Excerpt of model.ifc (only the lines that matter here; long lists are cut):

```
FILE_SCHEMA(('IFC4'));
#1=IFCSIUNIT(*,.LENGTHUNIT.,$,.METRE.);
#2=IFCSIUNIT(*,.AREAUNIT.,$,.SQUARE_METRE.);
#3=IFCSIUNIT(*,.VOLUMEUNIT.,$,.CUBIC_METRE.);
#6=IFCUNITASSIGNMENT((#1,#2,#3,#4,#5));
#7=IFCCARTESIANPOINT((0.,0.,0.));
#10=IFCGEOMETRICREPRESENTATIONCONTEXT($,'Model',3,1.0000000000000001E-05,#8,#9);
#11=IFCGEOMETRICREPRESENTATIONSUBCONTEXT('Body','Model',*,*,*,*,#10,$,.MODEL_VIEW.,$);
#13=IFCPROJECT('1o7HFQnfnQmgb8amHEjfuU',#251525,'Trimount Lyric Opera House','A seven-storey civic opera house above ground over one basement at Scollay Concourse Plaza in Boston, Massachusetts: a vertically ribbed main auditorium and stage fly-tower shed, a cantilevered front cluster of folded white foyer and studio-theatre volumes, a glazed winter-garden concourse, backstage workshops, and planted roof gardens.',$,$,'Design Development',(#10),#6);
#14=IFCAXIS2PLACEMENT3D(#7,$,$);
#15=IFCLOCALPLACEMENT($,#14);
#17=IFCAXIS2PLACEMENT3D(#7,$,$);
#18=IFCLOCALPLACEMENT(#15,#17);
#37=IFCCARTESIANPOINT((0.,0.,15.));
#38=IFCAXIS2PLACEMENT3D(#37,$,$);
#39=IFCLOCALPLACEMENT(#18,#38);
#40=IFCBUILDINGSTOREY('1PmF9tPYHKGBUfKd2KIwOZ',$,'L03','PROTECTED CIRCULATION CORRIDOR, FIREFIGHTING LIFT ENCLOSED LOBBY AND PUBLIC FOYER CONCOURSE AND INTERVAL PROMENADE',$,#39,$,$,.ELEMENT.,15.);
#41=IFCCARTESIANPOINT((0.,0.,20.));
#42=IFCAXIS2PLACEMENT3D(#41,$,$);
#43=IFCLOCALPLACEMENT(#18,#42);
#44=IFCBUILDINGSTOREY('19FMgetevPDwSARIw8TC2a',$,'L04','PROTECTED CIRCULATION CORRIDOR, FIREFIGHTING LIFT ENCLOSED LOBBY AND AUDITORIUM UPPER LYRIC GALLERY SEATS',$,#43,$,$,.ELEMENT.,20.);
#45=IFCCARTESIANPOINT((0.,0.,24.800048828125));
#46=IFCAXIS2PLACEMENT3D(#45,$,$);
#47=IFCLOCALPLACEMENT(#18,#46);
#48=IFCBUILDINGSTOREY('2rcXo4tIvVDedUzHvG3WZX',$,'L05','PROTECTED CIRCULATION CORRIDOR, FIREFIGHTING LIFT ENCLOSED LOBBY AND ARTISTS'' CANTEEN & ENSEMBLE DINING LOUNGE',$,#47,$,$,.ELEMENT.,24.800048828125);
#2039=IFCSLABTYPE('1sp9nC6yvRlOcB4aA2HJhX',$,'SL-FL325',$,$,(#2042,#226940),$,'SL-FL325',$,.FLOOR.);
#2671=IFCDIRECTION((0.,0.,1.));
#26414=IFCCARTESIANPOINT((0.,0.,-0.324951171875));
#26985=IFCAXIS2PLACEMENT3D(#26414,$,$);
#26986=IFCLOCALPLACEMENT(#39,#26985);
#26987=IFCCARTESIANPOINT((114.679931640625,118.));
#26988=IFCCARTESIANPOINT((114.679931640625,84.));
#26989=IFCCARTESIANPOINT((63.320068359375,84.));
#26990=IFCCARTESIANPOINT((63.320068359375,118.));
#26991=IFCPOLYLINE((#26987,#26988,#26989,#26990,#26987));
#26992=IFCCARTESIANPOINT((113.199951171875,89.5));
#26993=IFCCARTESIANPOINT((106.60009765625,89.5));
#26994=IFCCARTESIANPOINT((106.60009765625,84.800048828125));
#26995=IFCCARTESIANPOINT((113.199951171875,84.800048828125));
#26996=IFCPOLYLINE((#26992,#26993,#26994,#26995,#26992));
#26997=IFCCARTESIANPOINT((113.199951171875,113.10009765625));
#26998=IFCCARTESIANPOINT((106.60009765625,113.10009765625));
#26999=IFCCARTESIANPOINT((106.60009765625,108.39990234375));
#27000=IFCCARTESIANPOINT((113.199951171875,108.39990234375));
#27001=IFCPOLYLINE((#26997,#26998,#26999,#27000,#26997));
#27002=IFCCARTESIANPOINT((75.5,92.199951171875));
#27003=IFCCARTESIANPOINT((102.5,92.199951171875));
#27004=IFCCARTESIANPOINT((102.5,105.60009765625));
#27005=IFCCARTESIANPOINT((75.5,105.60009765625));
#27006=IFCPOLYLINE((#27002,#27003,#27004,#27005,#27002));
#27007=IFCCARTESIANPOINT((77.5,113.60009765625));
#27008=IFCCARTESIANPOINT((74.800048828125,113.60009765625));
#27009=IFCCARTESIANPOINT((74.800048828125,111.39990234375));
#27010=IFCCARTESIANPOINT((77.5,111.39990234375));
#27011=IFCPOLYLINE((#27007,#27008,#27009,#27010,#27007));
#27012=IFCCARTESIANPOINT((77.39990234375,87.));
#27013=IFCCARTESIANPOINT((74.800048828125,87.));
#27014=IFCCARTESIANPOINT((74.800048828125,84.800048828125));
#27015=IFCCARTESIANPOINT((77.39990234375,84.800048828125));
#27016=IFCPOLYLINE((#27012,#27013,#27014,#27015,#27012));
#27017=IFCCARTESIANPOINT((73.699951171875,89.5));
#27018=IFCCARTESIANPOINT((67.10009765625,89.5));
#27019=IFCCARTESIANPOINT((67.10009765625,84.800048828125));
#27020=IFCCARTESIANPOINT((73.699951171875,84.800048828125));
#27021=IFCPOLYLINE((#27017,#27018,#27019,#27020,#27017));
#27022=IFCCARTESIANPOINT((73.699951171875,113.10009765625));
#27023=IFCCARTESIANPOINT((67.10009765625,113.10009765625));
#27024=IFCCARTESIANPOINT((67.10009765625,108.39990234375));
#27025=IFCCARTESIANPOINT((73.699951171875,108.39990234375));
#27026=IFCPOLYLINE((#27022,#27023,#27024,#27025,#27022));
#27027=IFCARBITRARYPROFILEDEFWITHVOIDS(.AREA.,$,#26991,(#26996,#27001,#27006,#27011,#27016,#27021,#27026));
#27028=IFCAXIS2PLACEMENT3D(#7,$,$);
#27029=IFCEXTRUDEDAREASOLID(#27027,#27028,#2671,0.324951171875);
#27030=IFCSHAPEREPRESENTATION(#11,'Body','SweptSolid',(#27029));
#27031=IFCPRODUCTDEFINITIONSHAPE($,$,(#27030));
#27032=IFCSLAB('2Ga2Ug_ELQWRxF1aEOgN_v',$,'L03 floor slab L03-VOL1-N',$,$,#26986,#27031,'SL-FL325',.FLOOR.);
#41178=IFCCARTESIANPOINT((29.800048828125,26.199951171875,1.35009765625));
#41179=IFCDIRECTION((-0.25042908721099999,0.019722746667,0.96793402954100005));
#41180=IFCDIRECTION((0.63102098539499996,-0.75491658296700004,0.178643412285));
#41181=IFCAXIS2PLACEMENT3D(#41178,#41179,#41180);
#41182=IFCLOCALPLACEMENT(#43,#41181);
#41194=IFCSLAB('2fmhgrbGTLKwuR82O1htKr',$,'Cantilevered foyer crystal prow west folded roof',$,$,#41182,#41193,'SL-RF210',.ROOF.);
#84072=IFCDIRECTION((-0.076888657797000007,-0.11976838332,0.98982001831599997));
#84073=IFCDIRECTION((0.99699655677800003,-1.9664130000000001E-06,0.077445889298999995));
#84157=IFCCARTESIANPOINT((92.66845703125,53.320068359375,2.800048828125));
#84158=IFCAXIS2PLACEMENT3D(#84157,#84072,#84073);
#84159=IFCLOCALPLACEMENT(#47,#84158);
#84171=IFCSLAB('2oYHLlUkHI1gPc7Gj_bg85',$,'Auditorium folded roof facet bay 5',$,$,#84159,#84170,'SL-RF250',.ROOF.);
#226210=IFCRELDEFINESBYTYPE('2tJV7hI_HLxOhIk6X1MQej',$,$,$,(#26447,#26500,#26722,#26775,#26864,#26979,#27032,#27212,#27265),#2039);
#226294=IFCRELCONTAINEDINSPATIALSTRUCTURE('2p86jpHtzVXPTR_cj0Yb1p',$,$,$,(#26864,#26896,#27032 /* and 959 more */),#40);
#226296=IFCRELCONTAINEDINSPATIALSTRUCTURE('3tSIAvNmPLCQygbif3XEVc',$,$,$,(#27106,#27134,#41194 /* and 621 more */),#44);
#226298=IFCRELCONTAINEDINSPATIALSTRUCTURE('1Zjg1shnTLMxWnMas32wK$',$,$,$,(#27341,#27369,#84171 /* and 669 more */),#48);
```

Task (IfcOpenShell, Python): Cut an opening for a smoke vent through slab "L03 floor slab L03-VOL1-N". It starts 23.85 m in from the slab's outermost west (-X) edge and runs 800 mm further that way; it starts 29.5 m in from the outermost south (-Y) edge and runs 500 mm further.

```python
import numpy as np
import ifcopenshell
import ifcopenshell.api.feature
import ifcopenshell.api.geometry
import ifcopenshell.api.root
import ifcopenshell.geom
import ifcopenshell.util.placement
import ifcopenshell.util.representation
import ifcopenshell.util.shape
import ifcopenshell.util.unit

model = ifcopenshell.open("model.ifc")
unit_scale = ifcopenshell.util.unit.calculate_unit_scale(model)
settings = ifcopenshell.geom.settings()


def volume(element):
    """Net volume in cubic metres, openings subtracted."""
    shape = ifcopenshell.geom.create_shape(settings, element)
    return ifcopenshell.util.shape.get_volume(shape.geometry)


slab = model.by_guid("2Ga2Ug_ELQWRxF1aEOgN_v")
before = volume(slab)

# Extent in the slab's own axes, in metres. The edges named are its -X and -Y sides.
slab_shape = ifcopenshell.geom.create_shape(settings, slab)
vertices = ifcopenshell.util.shape.get_vertices(slab_shape.geometry)
x_min, y_min, bottom = vertices.min(axis=0)
top = vertices[:, 2].max()

opening = ifcopenshell.api.root.create_entity(model, ifc_class="IfcOpeningElement", name="Smoke vent opening", predefined_type="OPENING")
context = ifcopenshell.util.representation.get_context(model, "Model", "Body", "MODEL_VIEW")
width, depth = 0.8, 0.5
outline = [(0.0, 0.0), (width, 0.0), (width, depth), (0.0, depth), (0.0, 0.0)]
# Overshoot both faces by 50 mm so the cut is clean.
shape = ifcopenshell.api.geometry.add_slab_representation(
    model, context=context, depth=top - bottom + 0.1, polyline=outline
)
ifcopenshell.api.geometry.assign_representation(model, product=opening, representation=shape)

matrix = ifcopenshell.util.placement.get_local_placement(slab.ObjectPlacement)
matrix[:, 3] = matrix @ np.append(np.array([x_min + 23.85, y_min + 29.5, bottom - 0.05]) / unit_scale, 1.0)
ifcopenshell.api.geometry.edit_object_placement(model, product=opening, matrix=matrix, is_si=False)
ifcopenshell.api.feature.add_feature(model, feature=opening, element=slab)

after = volume(slab)

print(f"slab volume {before:.3f} -> {after:.3f} m3")

model.write("model_v2.ifc")
```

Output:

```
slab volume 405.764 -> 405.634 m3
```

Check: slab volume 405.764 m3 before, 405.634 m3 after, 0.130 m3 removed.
